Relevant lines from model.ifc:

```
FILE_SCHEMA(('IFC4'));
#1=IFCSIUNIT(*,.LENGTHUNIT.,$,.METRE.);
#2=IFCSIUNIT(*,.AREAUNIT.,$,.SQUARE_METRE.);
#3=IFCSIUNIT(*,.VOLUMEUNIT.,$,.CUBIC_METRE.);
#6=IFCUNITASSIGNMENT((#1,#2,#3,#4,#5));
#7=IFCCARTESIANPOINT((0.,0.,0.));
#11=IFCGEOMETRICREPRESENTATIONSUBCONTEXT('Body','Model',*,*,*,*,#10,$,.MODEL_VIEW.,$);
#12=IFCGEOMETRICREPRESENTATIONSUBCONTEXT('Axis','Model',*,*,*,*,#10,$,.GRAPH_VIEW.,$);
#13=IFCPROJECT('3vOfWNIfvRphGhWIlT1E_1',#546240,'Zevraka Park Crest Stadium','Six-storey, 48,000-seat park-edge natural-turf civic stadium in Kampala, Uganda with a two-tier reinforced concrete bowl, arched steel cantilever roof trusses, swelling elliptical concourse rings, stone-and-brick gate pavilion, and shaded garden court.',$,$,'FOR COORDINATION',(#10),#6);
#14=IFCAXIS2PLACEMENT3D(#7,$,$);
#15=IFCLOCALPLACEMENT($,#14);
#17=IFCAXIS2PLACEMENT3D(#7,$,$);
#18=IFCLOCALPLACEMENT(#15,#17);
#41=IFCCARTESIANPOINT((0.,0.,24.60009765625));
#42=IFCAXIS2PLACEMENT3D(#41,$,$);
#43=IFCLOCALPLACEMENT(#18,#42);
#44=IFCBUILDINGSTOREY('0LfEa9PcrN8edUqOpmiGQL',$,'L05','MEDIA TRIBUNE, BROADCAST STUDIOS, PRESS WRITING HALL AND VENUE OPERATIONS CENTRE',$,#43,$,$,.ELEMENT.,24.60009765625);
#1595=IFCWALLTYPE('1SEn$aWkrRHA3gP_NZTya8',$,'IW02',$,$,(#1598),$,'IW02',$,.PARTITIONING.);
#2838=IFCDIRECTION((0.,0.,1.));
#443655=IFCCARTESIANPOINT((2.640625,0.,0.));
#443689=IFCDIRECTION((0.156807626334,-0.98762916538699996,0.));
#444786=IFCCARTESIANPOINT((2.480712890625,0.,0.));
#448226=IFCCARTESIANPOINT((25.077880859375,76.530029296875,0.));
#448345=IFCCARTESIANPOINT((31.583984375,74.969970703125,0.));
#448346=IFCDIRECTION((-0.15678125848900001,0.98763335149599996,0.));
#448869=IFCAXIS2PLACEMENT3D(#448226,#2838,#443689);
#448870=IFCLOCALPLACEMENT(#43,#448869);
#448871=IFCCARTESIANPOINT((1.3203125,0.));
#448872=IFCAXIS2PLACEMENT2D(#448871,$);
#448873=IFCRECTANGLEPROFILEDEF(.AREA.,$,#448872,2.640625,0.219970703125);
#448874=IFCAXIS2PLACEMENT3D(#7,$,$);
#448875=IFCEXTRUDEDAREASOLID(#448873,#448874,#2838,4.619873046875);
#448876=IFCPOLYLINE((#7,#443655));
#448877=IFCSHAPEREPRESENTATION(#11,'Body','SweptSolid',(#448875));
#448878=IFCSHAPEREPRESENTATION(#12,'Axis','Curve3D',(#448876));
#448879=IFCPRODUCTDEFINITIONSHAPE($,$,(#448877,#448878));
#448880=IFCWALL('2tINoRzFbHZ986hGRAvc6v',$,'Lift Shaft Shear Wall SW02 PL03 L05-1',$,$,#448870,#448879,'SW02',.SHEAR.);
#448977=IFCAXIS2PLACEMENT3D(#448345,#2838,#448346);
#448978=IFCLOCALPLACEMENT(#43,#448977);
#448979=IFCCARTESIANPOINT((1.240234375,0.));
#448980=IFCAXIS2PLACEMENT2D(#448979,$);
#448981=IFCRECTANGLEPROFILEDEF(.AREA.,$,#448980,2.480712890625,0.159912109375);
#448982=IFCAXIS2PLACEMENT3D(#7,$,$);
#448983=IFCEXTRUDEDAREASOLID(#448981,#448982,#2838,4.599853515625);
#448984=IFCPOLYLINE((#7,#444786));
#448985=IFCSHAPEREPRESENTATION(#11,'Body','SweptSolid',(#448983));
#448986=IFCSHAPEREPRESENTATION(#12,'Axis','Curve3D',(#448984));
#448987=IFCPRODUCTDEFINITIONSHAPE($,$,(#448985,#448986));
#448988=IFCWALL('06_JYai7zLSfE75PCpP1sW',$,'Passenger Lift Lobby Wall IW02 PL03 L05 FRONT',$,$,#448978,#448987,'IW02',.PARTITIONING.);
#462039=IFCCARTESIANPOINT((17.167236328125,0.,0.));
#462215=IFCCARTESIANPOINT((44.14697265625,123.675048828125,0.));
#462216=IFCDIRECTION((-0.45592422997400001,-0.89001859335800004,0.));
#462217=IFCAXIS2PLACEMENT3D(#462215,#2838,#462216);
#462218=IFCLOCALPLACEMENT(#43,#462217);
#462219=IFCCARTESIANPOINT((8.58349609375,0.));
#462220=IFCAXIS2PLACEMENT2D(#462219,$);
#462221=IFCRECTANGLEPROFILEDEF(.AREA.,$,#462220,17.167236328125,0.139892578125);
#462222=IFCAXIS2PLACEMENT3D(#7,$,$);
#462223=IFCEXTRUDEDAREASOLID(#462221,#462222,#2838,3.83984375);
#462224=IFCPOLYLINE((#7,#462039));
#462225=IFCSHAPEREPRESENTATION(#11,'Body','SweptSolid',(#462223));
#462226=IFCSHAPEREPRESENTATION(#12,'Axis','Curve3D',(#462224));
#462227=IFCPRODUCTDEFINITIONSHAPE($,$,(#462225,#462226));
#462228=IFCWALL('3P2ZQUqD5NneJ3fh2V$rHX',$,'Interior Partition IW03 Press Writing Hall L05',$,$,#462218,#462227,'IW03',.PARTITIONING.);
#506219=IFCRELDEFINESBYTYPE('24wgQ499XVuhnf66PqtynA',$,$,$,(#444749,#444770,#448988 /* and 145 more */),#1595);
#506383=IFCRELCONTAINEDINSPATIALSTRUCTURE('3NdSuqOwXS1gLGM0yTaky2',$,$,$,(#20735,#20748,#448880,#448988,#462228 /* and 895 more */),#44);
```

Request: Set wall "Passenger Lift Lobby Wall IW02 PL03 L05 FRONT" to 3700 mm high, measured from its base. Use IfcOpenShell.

```python
import ifcopenshell
import ifcopenshell.geom
import ifcopenshell.util.representation
import ifcopenshell.util.shape

model = ifcopenshell.open("model.ifc")
settings = ifcopenshell.geom.settings()


def volume(element):
    """Net volume in cubic metres, openings subtracted."""
    shape = ifcopenshell.geom.create_shape(settings, element)
    return ifcopenshell.util.shape.get_volume(shape.geometry)


wall = model.by_guid("06_JYai7zLSfE75PCpP1sW")
before = volume(wall)

body = ifcopenshell.util.representation.get_representation(wall, "Model", "Body")
solid = body.Items[0]
old_height = solid.Depth
solid.Depth = 3.7
after = volume(wall)

print(f"height {old_height:g} -> {solid.Depth:g}, volume {before:.3f} -> {after:.3f} m3")

model.write("model_edited.ifc")
```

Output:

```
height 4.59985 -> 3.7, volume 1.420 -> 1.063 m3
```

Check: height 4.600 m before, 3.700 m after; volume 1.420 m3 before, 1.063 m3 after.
